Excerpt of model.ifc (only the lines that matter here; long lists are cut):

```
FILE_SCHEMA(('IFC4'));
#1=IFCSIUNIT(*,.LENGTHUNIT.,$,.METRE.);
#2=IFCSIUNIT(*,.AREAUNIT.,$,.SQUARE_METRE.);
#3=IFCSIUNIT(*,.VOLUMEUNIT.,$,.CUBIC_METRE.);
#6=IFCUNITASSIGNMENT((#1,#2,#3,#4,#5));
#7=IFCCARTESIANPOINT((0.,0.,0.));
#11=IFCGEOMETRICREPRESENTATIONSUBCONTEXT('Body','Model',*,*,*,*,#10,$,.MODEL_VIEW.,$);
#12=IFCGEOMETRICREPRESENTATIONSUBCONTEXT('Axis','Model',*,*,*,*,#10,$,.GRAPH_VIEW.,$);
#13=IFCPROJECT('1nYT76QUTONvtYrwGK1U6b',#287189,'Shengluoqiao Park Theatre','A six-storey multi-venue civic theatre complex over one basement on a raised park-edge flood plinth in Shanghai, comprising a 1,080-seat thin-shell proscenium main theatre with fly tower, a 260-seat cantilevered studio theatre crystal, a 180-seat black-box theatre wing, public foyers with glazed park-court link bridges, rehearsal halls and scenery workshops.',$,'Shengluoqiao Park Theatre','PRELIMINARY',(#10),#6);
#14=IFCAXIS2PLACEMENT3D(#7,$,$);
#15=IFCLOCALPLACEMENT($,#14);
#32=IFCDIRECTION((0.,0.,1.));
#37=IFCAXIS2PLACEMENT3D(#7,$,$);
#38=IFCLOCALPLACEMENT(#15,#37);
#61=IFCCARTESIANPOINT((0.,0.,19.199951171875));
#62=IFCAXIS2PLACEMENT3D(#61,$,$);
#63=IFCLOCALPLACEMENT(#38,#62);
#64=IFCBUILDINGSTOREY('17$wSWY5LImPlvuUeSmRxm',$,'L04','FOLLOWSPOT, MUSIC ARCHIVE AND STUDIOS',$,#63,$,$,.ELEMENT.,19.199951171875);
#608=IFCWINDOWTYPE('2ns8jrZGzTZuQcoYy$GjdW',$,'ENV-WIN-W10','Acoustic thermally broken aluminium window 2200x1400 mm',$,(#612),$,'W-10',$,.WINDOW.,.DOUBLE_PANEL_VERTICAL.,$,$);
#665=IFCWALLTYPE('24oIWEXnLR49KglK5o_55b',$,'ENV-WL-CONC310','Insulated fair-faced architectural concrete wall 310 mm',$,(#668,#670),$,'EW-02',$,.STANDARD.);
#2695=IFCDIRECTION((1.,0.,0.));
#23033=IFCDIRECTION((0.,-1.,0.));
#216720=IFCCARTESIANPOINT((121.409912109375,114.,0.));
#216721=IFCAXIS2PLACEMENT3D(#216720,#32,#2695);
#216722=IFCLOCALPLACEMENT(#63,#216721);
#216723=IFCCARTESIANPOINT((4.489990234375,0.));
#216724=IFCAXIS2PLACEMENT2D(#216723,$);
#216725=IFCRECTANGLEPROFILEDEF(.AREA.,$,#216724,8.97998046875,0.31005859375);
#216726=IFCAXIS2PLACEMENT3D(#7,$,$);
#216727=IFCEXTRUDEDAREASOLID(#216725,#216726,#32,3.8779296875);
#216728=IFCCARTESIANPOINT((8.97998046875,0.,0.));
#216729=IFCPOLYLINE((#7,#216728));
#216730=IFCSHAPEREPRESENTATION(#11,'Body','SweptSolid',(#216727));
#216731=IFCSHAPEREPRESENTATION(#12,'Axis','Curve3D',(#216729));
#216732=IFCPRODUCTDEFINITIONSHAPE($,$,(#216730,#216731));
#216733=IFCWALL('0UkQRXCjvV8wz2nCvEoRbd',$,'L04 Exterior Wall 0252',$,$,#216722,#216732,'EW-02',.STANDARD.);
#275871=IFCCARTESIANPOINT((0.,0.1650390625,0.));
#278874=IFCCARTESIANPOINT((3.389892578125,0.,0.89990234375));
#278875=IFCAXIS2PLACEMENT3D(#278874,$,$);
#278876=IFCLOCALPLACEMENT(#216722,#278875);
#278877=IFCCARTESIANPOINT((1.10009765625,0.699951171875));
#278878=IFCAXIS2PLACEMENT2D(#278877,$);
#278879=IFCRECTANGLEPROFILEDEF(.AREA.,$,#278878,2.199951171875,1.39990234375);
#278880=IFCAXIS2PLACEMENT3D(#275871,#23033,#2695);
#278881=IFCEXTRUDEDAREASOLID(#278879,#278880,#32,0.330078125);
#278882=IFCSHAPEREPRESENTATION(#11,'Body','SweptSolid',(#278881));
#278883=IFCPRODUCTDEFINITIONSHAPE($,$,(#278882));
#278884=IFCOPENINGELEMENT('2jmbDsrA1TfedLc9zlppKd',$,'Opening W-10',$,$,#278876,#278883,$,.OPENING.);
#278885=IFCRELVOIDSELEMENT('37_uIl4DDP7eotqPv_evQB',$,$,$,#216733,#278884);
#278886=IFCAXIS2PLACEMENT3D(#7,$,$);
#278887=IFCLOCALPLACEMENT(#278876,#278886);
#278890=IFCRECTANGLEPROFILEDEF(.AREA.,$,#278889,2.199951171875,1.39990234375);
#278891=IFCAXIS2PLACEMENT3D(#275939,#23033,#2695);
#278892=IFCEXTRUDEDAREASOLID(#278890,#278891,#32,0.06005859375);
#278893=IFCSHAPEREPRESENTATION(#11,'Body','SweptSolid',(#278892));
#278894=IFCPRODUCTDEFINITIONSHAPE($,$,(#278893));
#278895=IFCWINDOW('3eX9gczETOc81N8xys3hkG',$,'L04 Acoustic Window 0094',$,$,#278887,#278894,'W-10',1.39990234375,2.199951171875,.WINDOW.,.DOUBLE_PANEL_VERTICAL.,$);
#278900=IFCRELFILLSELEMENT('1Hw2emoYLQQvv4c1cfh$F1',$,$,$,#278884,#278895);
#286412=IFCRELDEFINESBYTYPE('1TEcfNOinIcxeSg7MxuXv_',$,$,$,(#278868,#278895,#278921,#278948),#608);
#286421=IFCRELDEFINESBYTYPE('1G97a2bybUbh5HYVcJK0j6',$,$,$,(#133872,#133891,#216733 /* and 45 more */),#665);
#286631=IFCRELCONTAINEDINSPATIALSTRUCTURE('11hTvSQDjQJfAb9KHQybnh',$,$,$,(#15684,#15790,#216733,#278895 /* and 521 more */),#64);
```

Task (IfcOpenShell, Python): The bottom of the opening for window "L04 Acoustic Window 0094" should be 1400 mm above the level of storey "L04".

```python
import numpy as np
import ifcopenshell
import ifcopenshell.api.geometry
import ifcopenshell.geom
import ifcopenshell.util.element
import ifcopenshell.util.placement
import ifcopenshell.util.shape
import ifcopenshell.util.unit

model = ifcopenshell.open("model.ifc")
unit_scale = ifcopenshell.util.unit.calculate_unit_scale(model)

window = model.by_guid("3eX9gczETOc81N8xys3hkG")
opening = window.FillsVoids[0].RelatingOpeningElement
storey = ifcopenshell.util.element.get_container(window, ifc_class="IfcBuildingStorey")
level = ifcopenshell.util.placement.get_local_placement(storey.ObjectPlacement)[2, 3]

# The opening's origin need not be at the sill, so measure its lowest point.
shape = ifcopenshell.geom.create_shape(ifcopenshell.geom.settings(), opening)
bottom = ifcopenshell.util.shape.get_shape_bottom_elevation(shape, shape.geometry) / unit_scale
dz = level + 1.4 / unit_scale - bottom

shift = np.array([0.0, 0.0, dz])
# The window is placed relative to its opening, so it follows when the opening moves.
matrix = ifcopenshell.util.placement.get_local_placement(opening.ObjectPlacement)
matrix[:3, 3] += shift
ifcopenshell.api.geometry.edit_object_placement(
    model, product=opening, matrix=matrix, is_si=False, should_transform_children=True
)

print(f"moved by {dz * unit_scale:+.3f} m")

model.write("model_rev.ifc")
```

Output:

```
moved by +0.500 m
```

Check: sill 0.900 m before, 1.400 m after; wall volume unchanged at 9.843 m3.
